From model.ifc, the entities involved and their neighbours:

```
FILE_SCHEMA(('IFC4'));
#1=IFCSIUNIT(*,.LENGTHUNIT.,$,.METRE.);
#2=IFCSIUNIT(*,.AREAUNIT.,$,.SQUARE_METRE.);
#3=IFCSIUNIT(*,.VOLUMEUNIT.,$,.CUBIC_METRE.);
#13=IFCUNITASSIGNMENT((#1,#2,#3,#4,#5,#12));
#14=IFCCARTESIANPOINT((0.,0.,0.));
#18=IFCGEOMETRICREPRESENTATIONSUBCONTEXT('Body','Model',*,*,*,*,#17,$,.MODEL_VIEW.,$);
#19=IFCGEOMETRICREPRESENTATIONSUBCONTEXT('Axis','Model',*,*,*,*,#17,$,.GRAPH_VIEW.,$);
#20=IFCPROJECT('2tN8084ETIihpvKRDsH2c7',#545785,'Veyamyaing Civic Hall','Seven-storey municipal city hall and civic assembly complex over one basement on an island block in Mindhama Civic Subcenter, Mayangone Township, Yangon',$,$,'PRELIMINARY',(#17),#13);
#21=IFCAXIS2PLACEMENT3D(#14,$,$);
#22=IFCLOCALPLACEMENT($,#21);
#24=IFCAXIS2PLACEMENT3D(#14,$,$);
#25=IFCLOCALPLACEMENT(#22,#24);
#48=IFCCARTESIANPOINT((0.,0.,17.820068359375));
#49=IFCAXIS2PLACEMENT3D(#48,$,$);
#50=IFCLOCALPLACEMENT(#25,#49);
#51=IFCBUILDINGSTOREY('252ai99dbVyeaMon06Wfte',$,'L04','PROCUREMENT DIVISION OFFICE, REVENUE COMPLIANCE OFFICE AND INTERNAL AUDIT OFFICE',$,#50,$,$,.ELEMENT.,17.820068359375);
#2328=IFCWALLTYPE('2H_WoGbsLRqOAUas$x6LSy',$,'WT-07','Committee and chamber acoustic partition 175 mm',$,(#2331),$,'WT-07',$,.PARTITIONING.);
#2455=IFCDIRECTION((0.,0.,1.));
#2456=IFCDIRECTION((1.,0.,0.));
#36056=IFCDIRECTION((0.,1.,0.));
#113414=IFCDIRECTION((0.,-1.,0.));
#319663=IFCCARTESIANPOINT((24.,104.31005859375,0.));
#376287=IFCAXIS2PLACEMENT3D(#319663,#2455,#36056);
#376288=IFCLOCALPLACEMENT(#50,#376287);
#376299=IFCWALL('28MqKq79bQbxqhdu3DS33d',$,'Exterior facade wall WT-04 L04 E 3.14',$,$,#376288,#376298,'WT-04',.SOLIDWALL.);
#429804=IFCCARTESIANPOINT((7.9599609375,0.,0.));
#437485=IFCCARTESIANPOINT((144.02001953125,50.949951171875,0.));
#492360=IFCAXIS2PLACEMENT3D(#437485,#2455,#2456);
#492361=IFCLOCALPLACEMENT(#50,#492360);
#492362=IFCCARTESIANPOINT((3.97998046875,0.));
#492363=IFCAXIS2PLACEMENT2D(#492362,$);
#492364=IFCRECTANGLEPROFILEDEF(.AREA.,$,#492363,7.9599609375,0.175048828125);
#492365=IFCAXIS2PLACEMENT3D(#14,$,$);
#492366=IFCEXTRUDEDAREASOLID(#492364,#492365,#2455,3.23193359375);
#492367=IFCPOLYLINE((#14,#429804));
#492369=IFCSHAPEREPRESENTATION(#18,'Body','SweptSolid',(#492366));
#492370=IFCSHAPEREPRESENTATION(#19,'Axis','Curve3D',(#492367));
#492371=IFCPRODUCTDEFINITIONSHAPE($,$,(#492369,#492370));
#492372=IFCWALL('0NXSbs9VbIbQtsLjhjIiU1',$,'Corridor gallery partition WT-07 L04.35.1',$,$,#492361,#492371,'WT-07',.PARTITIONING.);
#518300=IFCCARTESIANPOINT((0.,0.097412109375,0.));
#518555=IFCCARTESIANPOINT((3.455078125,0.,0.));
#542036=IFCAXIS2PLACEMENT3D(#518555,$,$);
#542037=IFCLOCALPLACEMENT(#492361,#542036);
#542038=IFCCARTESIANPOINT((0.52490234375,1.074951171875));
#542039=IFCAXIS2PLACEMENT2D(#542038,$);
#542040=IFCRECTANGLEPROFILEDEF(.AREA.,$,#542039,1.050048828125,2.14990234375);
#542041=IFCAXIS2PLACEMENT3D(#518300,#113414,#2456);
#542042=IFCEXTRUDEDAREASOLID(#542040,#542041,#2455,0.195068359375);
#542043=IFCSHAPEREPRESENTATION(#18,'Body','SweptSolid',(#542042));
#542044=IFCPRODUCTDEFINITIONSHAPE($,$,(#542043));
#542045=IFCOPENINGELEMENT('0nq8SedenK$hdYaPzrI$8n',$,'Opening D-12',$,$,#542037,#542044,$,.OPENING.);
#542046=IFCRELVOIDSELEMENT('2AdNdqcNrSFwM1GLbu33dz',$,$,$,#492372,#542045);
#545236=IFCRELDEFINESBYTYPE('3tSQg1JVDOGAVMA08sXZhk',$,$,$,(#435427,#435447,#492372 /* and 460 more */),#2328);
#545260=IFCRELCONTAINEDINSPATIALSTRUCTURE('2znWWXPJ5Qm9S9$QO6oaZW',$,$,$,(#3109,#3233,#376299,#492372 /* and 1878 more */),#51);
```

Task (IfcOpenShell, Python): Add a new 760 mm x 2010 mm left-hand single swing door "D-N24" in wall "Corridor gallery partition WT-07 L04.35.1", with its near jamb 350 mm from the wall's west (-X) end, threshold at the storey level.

```python
import numpy as np
import ifcopenshell
import ifcopenshell.api.feature
import ifcopenshell.api.geometry
import ifcopenshell.api.root
import ifcopenshell.api.spatial
import ifcopenshell.geom
import ifcopenshell.util.element
import ifcopenshell.util.placement
import ifcopenshell.util.representation
import ifcopenshell.util.shape
import ifcopenshell.util.unit

model = ifcopenshell.open("model.ifc")
unit_scale = ifcopenshell.util.unit.calculate_unit_scale(model)
settings = ifcopenshell.geom.settings()


def volume(element):
    """Net volume in cubic metres, openings subtracted."""
    shape = ifcopenshell.geom.create_shape(settings, element)
    return ifcopenshell.util.shape.get_volume(shape.geometry)


wall = model.by_id(492372)
storey = ifcopenshell.util.element.get_container(wall, ifc_class="IfcBuildingStorey")
context = ifcopenshell.util.representation.get_context(model, "Model", "Body", "MODEL_VIEW")
before = volume(wall)

width, height, from_end, sill = 0.76, 2.01, 0.35, 0.0  # metres

# The wall runs along its own X axis, and the end named is its -X end.
wall_shape = ifcopenshell.geom.create_shape(settings, wall)
x, y, z = ifcopenshell.util.shape.get_vertices(wall_shape.geometry).T
start = x.min() + from_end
face, thickness = float(y.min()), float(y.max() - y.min())
wall_matrix = ifcopenshell.util.placement.get_local_placement(wall.ObjectPlacement)
level = ifcopenshell.util.placement.get_local_placement(storey.ObjectPlacement)[2, 3]


def in_wall(x, y):
    """Placement at x, y metres in the wall's axes, at sill height."""
    matrix = wall_matrix.copy()
    matrix[:, 3] = wall_matrix @ np.array([x / unit_scale, y / unit_scale, 0.0, 1.0])
    matrix[2, 3] = level + sill / unit_scale
    return matrix


# Opening: a box that overshoots both wall faces by 50 mm.
opening = ifcopenshell.api.root.create_entity(model, ifc_class="IfcOpeningElement", predefined_type="OPENING")
box = ifcopenshell.api.geometry.add_wall_representation(
    model, context=context, length=width, height=height, thickness=thickness + 0.1
)
ifcopenshell.api.geometry.assign_representation(model, product=opening, representation=box)
ifcopenshell.api.geometry.edit_object_placement(model, product=opening, matrix=in_wall(start, face - 0.05), is_si=False)
ifcopenshell.api.feature.add_feature(model, feature=opening, element=wall)

door = ifcopenshell.api.root.create_entity(model, ifc_class="IfcDoor", name="D-N24", predefined_type="DOOR")
door.OverallWidth, door.OverallHeight = width / unit_scale, height / unit_scale
door.OperationType = "SINGLE_SWING_LEFT"
body = ifcopenshell.api.geometry.add_door_representation(
    model,
    context=context,
    overall_width=door.OverallWidth,
    overall_height=door.OverallHeight,
    operation_type="SINGLE_SWING_LEFT",
    lining_properties={"LiningDepth": thickness / unit_scale, "ThresholdDepth": thickness / unit_scale},
)
ifcopenshell.api.geometry.assign_representation(model, product=door, representation=body)
ifcopenshell.api.spatial.assign_container(model, products=[door], relating_structure=storey)
ifcopenshell.api.feature.add_filling(model, opening=opening, element=door)

# The lining spans the wall, so the door starts at the wall face.
ifcopenshell.api.geometry.edit_object_placement(model, product=door, matrix=in_wall(start, face), is_si=False)

after = volume(wall)

print(f"wall volume {before:.3f} -> {after:.3f} m3")

model.write("model_rev.ifc")
```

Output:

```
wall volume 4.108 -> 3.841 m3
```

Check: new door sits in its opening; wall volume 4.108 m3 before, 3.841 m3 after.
